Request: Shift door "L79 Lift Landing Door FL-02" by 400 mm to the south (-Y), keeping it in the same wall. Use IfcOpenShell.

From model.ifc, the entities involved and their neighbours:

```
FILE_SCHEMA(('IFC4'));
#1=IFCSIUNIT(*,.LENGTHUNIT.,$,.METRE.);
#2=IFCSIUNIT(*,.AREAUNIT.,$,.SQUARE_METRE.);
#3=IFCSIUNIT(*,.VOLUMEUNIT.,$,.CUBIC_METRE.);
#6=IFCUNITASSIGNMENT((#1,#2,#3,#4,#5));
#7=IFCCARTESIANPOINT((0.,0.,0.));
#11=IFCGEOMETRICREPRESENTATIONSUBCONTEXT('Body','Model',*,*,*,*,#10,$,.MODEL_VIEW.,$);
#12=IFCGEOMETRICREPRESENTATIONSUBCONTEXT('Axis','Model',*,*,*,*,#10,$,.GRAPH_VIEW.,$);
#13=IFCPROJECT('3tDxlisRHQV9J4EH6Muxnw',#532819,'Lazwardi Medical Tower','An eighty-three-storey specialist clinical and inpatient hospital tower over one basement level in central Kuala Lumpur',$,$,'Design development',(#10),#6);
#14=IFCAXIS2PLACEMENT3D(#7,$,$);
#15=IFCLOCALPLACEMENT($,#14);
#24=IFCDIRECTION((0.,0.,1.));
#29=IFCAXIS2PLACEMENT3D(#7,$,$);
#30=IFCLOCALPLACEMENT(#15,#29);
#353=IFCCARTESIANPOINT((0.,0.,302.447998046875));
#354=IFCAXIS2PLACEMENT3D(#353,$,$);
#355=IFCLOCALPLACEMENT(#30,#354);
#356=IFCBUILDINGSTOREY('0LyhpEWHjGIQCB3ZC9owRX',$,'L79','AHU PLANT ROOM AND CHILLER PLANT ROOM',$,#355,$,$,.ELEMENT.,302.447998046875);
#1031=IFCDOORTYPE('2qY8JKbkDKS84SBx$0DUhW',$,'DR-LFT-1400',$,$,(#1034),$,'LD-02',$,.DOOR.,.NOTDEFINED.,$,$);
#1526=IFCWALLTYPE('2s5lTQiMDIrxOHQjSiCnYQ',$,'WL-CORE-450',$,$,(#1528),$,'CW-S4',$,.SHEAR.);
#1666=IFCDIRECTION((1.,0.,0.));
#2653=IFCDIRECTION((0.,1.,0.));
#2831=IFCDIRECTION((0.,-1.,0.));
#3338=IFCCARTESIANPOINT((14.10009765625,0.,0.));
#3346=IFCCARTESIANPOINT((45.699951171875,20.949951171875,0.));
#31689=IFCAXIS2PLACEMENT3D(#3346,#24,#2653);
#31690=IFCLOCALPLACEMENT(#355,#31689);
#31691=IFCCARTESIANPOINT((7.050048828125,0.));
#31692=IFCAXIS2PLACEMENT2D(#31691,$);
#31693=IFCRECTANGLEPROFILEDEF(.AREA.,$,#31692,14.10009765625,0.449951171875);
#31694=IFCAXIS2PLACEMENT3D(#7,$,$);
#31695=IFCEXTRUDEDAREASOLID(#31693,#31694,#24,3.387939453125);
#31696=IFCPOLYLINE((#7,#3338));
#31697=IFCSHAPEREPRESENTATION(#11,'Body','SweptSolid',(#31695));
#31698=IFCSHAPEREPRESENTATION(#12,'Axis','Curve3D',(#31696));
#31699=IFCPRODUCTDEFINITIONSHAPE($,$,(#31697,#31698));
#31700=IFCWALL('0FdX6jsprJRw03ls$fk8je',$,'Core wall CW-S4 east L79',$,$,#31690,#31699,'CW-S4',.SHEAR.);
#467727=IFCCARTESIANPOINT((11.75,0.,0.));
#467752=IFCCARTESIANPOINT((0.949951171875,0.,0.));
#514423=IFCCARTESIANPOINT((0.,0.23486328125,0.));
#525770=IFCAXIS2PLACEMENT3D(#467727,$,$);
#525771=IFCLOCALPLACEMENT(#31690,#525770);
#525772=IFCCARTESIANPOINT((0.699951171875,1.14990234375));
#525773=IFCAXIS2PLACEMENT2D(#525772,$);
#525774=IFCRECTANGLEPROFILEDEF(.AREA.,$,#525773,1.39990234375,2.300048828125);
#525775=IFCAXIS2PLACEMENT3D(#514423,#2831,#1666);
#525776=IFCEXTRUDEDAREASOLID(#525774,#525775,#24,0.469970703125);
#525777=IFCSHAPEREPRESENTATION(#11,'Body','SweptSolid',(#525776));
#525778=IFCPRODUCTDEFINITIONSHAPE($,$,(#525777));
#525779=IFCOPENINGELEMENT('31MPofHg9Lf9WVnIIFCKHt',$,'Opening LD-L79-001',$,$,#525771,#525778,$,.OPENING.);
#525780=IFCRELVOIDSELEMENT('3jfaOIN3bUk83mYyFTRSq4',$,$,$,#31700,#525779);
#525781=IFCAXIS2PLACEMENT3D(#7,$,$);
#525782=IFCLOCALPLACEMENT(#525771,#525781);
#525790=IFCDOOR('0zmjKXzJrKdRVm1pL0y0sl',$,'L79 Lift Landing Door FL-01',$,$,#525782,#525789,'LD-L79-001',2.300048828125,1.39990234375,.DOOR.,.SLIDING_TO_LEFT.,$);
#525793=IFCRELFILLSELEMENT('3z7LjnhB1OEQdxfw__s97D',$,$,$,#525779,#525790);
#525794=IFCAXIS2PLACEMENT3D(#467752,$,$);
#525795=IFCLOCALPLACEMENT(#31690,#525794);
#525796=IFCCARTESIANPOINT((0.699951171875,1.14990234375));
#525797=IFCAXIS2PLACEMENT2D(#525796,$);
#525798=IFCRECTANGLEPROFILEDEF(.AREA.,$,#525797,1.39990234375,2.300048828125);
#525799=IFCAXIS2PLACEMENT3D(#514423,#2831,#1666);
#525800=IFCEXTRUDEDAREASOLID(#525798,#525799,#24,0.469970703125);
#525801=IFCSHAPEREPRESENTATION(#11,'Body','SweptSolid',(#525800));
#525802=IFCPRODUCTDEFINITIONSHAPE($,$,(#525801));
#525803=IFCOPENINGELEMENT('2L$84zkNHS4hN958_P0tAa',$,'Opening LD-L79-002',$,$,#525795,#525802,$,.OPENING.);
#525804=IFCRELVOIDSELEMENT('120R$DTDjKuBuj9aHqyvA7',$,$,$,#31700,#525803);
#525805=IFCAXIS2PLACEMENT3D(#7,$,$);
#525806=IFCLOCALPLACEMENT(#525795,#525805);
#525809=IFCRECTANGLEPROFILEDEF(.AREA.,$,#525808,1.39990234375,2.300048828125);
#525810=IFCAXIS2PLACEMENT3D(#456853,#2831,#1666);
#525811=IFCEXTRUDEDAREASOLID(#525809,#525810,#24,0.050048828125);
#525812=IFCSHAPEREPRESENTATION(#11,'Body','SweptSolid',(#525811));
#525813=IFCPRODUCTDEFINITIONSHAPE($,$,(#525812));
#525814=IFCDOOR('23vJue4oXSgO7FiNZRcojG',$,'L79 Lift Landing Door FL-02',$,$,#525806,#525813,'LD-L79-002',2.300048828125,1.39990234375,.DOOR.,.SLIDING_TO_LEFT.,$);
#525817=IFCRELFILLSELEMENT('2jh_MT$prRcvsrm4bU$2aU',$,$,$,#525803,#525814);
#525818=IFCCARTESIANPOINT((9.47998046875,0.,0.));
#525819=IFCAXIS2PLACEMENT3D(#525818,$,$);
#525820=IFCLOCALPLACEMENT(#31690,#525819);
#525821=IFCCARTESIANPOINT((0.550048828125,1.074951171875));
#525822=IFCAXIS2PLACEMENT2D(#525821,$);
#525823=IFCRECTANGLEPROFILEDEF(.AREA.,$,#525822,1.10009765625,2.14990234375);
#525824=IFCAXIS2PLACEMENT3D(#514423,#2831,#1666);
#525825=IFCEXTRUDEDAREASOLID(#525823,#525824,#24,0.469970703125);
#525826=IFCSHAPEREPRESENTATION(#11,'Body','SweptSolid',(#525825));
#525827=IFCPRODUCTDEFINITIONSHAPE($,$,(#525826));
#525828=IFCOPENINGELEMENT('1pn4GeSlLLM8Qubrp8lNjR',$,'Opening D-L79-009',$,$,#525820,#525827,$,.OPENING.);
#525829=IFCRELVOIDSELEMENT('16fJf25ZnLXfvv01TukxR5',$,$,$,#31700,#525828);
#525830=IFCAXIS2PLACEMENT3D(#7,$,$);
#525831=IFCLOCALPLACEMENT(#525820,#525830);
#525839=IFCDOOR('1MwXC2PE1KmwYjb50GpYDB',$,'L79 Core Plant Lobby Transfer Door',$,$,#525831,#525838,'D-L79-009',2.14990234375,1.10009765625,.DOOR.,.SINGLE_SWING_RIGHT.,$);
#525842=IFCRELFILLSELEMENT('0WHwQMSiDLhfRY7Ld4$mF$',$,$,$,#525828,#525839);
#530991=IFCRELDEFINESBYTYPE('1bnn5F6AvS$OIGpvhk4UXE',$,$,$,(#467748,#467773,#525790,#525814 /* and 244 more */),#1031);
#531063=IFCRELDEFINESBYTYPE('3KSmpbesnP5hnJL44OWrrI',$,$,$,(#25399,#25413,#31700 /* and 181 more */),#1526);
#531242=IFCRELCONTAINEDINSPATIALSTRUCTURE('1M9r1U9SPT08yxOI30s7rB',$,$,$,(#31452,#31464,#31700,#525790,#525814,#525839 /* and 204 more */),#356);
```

```python
import ifcopenshell
import ifcopenshell.api.geometry
import ifcopenshell.util.placement

model = ifcopenshell.open("model.ifc")

door = model.by_guid("23vJue4oXSgO7FiNZRcojG")
opening = door.FillsVoids[0].RelatingOpeningElement
wall = opening.VoidsElements[0].RelatingBuildingElement

wall_matrix = ifcopenshell.util.placement.get_local_placement(wall.ObjectPlacement)
shift = wall_matrix[:3, 0] * -0.4
before = ifcopenshell.util.placement.get_local_placement(door.ObjectPlacement)[:3, 3].copy()

# The door is placed relative to its opening, so it follows when the opening moves.
matrix = ifcopenshell.util.placement.get_local_placement(opening.ObjectPlacement)
matrix[:3, 3] += shift
ifcopenshell.api.geometry.edit_object_placement(
    model, product=opening, matrix=matrix, is_si=False, should_transform_children=True
)

after = ifcopenshell.util.placement.get_local_placement(door.ObjectPlacement)[:3, 3]
print("door moved by", (after - before).round(3) + 0.0)

model.write("model_rev.ifc")
```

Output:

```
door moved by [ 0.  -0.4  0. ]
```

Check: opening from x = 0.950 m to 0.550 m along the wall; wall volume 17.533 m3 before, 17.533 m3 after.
